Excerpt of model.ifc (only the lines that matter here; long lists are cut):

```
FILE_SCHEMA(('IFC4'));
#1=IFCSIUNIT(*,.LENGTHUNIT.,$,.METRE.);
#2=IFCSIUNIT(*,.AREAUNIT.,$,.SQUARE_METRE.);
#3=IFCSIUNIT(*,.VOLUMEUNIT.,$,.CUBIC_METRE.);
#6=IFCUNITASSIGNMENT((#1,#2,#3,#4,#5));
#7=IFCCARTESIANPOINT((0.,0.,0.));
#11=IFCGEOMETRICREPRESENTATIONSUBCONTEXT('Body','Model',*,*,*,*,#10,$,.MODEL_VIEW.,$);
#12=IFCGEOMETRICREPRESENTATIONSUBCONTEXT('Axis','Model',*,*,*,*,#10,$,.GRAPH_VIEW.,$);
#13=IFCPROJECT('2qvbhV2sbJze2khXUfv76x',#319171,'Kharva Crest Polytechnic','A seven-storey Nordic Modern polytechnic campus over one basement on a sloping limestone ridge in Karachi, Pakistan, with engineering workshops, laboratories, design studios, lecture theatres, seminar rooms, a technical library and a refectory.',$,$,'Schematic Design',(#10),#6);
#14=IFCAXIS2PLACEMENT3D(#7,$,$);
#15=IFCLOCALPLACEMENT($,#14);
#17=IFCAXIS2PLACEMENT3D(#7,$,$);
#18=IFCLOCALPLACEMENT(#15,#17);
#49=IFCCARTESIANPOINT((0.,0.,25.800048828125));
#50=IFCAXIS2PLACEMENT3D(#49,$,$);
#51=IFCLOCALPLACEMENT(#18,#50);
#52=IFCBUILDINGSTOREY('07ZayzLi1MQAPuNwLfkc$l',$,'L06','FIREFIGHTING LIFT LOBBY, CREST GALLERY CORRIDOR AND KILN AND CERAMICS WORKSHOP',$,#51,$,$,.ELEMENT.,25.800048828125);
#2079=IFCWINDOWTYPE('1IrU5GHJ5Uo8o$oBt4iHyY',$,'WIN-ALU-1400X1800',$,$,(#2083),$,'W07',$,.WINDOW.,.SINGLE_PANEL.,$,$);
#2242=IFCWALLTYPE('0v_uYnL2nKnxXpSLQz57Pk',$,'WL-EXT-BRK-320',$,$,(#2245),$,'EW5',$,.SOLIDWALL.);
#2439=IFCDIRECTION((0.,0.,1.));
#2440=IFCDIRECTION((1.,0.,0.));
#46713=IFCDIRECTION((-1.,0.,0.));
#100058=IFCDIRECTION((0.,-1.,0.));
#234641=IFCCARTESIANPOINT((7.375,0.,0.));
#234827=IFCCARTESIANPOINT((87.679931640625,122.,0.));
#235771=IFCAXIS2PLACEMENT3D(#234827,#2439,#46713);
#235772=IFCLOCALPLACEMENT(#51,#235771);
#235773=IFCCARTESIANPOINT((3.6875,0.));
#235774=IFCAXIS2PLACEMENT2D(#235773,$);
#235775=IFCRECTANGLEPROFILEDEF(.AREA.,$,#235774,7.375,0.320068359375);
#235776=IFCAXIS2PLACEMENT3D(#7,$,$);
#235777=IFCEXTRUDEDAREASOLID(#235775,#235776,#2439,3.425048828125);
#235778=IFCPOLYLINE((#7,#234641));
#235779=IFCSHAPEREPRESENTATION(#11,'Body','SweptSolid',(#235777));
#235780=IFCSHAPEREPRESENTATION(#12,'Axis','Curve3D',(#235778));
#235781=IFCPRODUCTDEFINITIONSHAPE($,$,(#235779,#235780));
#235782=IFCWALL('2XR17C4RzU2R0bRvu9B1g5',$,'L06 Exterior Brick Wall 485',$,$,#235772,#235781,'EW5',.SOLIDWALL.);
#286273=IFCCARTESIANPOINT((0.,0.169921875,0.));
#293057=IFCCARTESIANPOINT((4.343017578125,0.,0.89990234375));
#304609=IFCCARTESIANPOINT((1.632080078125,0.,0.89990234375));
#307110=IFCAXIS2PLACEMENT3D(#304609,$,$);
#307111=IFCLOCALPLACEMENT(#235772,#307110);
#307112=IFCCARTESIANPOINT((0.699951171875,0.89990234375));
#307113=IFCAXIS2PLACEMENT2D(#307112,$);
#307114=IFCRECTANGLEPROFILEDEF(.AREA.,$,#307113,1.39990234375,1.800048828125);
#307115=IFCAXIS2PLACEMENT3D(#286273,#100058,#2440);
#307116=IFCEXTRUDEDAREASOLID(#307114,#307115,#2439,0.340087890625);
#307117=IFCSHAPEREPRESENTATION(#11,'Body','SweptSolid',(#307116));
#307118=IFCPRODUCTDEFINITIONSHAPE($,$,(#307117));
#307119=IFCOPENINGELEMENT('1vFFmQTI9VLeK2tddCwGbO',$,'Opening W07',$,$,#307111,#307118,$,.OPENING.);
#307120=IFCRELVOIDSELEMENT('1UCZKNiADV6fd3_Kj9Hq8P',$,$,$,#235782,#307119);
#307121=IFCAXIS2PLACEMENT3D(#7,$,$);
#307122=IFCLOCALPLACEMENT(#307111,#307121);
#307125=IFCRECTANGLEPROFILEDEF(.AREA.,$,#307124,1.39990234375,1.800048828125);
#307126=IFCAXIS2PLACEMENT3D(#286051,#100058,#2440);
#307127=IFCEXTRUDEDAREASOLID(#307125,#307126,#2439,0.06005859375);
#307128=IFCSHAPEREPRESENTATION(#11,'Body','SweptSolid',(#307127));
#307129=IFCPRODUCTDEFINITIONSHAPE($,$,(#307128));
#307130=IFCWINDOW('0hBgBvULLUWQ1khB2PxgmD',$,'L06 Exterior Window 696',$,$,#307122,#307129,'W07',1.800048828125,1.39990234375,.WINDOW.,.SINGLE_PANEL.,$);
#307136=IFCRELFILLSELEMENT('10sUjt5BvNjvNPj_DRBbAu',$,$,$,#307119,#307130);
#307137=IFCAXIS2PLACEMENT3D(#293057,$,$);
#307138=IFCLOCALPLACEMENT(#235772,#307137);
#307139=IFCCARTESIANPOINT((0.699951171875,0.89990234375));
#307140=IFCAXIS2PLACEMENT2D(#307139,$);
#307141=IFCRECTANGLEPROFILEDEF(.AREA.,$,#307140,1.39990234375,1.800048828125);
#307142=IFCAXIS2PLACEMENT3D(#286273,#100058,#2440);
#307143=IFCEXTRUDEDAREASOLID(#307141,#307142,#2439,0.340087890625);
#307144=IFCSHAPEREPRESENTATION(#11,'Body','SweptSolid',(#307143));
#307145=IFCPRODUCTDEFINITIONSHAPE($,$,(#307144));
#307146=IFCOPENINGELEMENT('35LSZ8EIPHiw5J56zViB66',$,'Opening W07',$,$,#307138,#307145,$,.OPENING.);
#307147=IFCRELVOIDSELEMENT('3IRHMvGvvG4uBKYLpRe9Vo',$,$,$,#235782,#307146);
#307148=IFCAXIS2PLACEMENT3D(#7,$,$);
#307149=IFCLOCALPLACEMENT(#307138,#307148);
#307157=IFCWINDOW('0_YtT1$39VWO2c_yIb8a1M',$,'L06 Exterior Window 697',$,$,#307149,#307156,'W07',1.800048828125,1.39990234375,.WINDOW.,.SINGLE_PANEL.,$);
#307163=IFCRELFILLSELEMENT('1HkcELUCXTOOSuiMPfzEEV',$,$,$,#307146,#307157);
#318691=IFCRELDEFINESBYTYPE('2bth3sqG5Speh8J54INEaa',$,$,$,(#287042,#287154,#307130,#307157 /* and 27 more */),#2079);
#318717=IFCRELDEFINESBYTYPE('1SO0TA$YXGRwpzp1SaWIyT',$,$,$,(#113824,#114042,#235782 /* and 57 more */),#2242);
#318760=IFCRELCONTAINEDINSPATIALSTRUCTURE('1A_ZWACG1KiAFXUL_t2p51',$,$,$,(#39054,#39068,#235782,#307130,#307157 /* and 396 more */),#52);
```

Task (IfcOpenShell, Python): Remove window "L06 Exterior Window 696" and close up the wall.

```python
import ifcopenshell
import ifcopenshell.api.feature
import ifcopenshell.api.root
import ifcopenshell.geom
import ifcopenshell.util.shape

model = ifcopenshell.open("model.ifc")
settings = ifcopenshell.geom.settings()


def volume(element):
    """Net volume in cubic metres, openings subtracted."""
    shape = ifcopenshell.geom.create_shape(settings, element)
    return ifcopenshell.util.shape.get_volume(shape.geometry)


window = model.by_guid("0hBgBvULLUWQ1khB2PxgmD")
opening = window.FillsVoids[0].RelatingOpeningElement
wall = opening.VoidsElements[0].RelatingBuildingElement
before = volume(wall)

ifcopenshell.api.root.remove_product(model, product=window)
ifcopenshell.api.feature.remove_feature(model, feature=opening)

after = volume(wall)

print(f"wall volume {before:.3f} -> {after:.3f} m3")

model.write("model_edited.ifc")
```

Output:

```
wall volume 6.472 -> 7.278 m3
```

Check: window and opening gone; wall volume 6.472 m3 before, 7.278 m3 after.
